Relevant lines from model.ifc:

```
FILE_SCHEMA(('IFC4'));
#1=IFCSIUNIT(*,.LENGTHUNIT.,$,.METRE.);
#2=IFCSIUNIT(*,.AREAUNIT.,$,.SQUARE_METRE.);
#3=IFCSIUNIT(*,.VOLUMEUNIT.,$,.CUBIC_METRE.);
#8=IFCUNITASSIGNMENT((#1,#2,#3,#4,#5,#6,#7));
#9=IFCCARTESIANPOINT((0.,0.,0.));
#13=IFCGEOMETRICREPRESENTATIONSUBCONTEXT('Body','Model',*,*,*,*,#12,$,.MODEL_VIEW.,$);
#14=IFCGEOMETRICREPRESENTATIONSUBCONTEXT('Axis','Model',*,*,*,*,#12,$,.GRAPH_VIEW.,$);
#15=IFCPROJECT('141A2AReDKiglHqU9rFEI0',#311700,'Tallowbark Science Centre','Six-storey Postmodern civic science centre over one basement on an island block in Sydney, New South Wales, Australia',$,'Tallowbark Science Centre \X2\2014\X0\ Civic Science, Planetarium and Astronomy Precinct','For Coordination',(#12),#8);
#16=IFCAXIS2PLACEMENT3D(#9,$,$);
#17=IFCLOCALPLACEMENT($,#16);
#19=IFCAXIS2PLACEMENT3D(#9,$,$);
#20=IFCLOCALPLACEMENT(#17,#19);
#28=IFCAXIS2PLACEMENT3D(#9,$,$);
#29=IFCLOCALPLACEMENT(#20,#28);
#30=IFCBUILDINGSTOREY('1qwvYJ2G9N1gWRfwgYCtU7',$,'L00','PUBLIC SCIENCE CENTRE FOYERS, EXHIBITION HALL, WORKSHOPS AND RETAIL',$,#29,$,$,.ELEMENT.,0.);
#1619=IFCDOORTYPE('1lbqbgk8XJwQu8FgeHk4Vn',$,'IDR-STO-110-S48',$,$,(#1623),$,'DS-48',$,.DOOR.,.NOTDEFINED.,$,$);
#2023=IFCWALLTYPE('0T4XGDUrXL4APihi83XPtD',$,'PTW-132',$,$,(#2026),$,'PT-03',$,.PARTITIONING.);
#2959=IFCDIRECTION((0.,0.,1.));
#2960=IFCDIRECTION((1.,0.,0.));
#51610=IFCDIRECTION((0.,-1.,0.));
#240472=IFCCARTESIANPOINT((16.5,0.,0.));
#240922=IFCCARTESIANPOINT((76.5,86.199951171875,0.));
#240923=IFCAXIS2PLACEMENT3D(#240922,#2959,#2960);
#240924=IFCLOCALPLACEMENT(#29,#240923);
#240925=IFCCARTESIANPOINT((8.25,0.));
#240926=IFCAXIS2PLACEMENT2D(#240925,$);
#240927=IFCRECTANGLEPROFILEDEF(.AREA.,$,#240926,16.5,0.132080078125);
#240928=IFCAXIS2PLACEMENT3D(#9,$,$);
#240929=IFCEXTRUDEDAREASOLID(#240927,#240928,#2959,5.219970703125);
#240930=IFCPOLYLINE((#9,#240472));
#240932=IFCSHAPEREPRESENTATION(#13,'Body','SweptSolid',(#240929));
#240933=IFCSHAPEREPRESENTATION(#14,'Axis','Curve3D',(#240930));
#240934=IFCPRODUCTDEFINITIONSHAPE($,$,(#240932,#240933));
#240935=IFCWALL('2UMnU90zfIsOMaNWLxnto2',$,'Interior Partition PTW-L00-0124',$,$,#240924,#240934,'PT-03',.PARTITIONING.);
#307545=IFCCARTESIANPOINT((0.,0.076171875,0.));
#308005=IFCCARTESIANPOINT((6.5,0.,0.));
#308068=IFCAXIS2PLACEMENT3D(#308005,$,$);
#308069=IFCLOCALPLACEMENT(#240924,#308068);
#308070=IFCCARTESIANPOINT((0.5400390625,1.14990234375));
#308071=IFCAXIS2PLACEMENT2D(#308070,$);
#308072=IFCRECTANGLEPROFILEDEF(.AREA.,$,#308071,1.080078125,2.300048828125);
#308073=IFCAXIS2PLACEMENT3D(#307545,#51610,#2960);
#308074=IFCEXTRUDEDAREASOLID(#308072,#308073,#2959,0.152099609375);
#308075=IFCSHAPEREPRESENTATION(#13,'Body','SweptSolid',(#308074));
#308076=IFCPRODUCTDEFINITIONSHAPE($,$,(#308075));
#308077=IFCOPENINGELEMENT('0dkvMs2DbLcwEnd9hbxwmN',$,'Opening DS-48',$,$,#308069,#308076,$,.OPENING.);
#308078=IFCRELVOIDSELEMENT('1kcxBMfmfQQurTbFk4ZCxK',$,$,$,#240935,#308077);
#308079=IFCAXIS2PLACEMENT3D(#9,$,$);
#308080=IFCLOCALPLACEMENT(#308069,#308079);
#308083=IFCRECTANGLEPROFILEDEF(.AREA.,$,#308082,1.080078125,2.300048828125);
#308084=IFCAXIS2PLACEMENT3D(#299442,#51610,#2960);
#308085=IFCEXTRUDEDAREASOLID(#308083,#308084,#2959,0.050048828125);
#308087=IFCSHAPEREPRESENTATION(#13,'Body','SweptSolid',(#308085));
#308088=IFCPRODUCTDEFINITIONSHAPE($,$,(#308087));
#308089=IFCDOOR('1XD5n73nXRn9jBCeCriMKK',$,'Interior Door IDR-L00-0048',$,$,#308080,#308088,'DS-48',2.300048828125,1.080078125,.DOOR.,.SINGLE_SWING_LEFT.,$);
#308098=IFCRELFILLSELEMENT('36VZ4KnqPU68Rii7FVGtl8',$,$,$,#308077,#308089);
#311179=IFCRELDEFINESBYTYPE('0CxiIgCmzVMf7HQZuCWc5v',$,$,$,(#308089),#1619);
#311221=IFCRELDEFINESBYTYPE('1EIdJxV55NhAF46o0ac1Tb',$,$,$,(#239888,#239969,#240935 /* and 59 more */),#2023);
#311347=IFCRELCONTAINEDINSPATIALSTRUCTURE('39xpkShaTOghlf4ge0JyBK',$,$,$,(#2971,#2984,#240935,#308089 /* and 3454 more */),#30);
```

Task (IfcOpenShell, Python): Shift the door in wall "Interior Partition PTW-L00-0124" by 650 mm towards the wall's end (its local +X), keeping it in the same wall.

```python
import ifcopenshell
import ifcopenshell.api.geometry
import ifcopenshell.util.placement

model = ifcopenshell.open("model.ifc")

door = model.by_guid("1XD5n73nXRn9jBCeCriMKK")
opening = door.FillsVoids[0].RelatingOpeningElement
wall = opening.VoidsElements[0].RelatingBuildingElement

wall_matrix = ifcopenshell.util.placement.get_local_placement(wall.ObjectPlacement)
shift = wall_matrix[:3, 0] * 0.65
before = ifcopenshell.util.placement.get_local_placement(door.ObjectPlacement)[:3, 3].copy()

# The door is placed relative to its opening, so it follows when the opening moves.
matrix = ifcopenshell.util.placement.get_local_placement(opening.ObjectPlacement)
matrix[:3, 3] += shift
ifcopenshell.api.geometry.edit_object_placement(
    model, product=opening, matrix=matrix, is_si=False, should_transform_children=True
)

after = ifcopenshell.util.placement.get_local_placement(door.ObjectPlacement)[:3, 3]
print("door moved by", (after - before).round(3) + 0.0)

model.write("model-out.ifc")
```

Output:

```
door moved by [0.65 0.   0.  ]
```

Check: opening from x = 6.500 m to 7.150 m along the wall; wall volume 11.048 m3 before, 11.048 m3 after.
